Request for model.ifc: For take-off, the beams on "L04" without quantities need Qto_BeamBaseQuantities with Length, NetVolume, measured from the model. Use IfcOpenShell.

First a look at what the model holds.

```python
import ifcopenshell
import ifcopenshell.util.element
import ifcopenshell.util.unit

model = ifcopenshell.open("model.ifc")
print(model.schema)
for unit_type in ("LENGTHUNIT", "AREAUNIT", "VOLUMEUNIT"):
    print(unit_type, ifcopenshell.util.unit.calculate_unit_scale(model, unit_type))
storey = next(s for s in model.by_type("IfcBuildingStorey") if s.Name == "L04")
beams = [e for e in ifcopenshell.util.element.get_decomposition(storey) if e.is_a("IfcBeam")]
for e in sorted(beams, key=lambda e: e.id()):
    print(e.id(), e.is_a(), e.Name, list(ifcopenshell.util.element.get_psets(e, qtos_only=True)), sep=" | ")
```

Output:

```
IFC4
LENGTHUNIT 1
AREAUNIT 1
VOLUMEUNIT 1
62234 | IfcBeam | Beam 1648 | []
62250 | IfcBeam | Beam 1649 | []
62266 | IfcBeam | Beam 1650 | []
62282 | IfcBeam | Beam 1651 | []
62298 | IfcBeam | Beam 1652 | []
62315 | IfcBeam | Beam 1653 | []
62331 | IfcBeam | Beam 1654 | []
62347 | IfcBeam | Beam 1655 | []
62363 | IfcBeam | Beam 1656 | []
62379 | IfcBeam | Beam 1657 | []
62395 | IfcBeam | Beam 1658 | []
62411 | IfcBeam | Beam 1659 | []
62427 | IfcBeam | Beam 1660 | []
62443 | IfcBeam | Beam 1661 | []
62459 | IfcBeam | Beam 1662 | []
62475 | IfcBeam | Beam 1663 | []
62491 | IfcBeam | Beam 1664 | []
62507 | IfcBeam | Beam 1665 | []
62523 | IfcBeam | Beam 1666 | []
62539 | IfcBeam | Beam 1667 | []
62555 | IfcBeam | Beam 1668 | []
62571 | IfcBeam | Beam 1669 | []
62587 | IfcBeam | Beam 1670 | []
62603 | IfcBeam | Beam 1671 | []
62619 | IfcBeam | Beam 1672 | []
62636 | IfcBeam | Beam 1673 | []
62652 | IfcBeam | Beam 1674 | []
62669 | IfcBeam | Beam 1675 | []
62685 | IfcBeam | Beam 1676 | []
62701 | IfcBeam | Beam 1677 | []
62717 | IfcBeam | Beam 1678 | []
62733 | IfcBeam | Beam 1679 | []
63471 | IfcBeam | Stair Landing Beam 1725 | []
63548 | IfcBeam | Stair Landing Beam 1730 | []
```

```python
import ifcopenshell
import ifcopenshell.api.pset
import ifcopenshell.geom
import ifcopenshell.util.element
import ifcopenshell.util.shape
import ifcopenshell.util.unit

model = ifcopenshell.open("model.ifc")
unit_scale = ifcopenshell.util.unit.calculate_unit_scale(model)
volume_scale = ifcopenshell.util.unit.calculate_unit_scale(model, "VOLUMEUNIT")
settings = ifcopenshell.geom.settings()

storey = next(s for s in model.by_type("IfcBuildingStorey") if s.Name == "L04")
beams = [e for e in ifcopenshell.util.element.get_decomposition(storey) if e.is_a("IfcBeam")]

for e in sorted(beams, key=lambda e: e.id()):
    if ifcopenshell.util.element.get_psets(e, qtos_only=True, should_inherit=False):
        continue
    # Geometry comes back in metres, in the element's own axes.
    shape = ifcopenshell.geom.create_shape(settings, e)
    values = {
        "Length": ifcopenshell.util.shape.get_max_xyz(shape.geometry) / unit_scale,
        "NetVolume": ifcopenshell.util.shape.get_volume(shape.geometry) / volume_scale,
    }
    qto = ifcopenshell.api.pset.add_qto(model, product=e, name="Qto_BeamBaseQuantities")
    ifcopenshell.api.pset.edit_qto(model, qto=qto, properties=values)
    print(e.id(), {k: round(v, 3) for k, v in values.items()})

model.write("model_updated.ifc")
```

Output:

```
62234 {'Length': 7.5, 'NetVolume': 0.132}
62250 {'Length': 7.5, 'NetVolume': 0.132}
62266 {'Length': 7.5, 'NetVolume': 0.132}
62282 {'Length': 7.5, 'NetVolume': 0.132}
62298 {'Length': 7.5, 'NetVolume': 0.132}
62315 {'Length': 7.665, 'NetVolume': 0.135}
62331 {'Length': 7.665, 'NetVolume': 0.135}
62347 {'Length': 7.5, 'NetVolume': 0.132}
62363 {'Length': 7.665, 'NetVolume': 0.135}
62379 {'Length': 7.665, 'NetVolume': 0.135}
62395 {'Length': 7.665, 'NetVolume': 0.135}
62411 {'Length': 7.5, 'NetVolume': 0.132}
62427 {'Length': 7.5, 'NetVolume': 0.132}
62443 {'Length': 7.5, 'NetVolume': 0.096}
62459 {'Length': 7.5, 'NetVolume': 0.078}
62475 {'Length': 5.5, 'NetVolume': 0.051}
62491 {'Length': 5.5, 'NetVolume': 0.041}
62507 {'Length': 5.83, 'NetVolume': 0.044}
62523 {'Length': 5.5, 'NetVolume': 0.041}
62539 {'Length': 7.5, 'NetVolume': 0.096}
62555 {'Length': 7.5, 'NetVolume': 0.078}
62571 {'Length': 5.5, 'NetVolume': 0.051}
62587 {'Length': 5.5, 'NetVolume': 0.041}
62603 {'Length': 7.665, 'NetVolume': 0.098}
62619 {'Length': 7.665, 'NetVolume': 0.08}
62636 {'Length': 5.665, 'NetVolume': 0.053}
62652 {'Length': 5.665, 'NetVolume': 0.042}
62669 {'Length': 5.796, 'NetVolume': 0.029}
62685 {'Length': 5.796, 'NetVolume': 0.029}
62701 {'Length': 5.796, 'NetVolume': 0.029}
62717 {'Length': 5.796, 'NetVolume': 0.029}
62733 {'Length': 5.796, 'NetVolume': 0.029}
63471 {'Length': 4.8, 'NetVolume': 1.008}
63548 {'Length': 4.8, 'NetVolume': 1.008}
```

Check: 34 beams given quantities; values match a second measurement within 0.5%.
